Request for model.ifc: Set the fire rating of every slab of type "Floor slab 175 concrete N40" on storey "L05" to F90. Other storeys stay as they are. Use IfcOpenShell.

First a look at what the model holds.

```python
import ifcopenshell
import ifcopenshell.util.element

model = ifcopenshell.open("model.ifc")
print(model.schema)
storey = next(s for s in model.by_type("IfcBuildingStorey") if s.Name == "L05")
slabs = [e for e in ifcopenshell.util.element.get_decomposition(storey) if e.is_a("IfcSlab")]
seen = {}
for e in slabs:
    element_type = ifcopenshell.util.element.get_type(e)
    key = (element_type.Name if element_type != e and element_type else None, ifcopenshell.util.element.get_pset(e, "Pset_SlabCommon", "FireRating"))
    seen[key] = seen.get(key, 0) + 1
for (name, value), count in sorted(seen.items(), key=str):
    print(count, "x", name, "|", value)
```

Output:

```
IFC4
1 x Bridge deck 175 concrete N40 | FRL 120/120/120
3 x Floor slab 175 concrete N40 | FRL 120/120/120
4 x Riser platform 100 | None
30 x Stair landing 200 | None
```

```python
import ifcopenshell
import ifcopenshell.api.pset
import ifcopenshell.util.element

model = ifcopenshell.open("model.ifc")

storey = next(s for s in model.by_type("IfcBuildingStorey") if s.Name == "L05")
slabs = [e for e in ifcopenshell.util.element.get_decomposition(storey) if e.is_a("IfcSlab")]

count = 0
for e in slabs:
    element_type = ifcopenshell.util.element.get_type(e)
    if element_type in (None, e) or element_type.Name != "Floor slab 175 concrete N40":
        continue
    # add_pset returns the element's existing set when there is one.
    pset = ifcopenshell.api.pset.add_pset(model, product=e, name="Pset_SlabCommon")
    ifcopenshell.api.pset.edit_pset(model, pset=pset, properties={"FireRating": "F90"})
    count += 1

print(count, "slabs updated")

model.write("model_rev.ifc")
```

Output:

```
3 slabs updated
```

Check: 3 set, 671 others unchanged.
